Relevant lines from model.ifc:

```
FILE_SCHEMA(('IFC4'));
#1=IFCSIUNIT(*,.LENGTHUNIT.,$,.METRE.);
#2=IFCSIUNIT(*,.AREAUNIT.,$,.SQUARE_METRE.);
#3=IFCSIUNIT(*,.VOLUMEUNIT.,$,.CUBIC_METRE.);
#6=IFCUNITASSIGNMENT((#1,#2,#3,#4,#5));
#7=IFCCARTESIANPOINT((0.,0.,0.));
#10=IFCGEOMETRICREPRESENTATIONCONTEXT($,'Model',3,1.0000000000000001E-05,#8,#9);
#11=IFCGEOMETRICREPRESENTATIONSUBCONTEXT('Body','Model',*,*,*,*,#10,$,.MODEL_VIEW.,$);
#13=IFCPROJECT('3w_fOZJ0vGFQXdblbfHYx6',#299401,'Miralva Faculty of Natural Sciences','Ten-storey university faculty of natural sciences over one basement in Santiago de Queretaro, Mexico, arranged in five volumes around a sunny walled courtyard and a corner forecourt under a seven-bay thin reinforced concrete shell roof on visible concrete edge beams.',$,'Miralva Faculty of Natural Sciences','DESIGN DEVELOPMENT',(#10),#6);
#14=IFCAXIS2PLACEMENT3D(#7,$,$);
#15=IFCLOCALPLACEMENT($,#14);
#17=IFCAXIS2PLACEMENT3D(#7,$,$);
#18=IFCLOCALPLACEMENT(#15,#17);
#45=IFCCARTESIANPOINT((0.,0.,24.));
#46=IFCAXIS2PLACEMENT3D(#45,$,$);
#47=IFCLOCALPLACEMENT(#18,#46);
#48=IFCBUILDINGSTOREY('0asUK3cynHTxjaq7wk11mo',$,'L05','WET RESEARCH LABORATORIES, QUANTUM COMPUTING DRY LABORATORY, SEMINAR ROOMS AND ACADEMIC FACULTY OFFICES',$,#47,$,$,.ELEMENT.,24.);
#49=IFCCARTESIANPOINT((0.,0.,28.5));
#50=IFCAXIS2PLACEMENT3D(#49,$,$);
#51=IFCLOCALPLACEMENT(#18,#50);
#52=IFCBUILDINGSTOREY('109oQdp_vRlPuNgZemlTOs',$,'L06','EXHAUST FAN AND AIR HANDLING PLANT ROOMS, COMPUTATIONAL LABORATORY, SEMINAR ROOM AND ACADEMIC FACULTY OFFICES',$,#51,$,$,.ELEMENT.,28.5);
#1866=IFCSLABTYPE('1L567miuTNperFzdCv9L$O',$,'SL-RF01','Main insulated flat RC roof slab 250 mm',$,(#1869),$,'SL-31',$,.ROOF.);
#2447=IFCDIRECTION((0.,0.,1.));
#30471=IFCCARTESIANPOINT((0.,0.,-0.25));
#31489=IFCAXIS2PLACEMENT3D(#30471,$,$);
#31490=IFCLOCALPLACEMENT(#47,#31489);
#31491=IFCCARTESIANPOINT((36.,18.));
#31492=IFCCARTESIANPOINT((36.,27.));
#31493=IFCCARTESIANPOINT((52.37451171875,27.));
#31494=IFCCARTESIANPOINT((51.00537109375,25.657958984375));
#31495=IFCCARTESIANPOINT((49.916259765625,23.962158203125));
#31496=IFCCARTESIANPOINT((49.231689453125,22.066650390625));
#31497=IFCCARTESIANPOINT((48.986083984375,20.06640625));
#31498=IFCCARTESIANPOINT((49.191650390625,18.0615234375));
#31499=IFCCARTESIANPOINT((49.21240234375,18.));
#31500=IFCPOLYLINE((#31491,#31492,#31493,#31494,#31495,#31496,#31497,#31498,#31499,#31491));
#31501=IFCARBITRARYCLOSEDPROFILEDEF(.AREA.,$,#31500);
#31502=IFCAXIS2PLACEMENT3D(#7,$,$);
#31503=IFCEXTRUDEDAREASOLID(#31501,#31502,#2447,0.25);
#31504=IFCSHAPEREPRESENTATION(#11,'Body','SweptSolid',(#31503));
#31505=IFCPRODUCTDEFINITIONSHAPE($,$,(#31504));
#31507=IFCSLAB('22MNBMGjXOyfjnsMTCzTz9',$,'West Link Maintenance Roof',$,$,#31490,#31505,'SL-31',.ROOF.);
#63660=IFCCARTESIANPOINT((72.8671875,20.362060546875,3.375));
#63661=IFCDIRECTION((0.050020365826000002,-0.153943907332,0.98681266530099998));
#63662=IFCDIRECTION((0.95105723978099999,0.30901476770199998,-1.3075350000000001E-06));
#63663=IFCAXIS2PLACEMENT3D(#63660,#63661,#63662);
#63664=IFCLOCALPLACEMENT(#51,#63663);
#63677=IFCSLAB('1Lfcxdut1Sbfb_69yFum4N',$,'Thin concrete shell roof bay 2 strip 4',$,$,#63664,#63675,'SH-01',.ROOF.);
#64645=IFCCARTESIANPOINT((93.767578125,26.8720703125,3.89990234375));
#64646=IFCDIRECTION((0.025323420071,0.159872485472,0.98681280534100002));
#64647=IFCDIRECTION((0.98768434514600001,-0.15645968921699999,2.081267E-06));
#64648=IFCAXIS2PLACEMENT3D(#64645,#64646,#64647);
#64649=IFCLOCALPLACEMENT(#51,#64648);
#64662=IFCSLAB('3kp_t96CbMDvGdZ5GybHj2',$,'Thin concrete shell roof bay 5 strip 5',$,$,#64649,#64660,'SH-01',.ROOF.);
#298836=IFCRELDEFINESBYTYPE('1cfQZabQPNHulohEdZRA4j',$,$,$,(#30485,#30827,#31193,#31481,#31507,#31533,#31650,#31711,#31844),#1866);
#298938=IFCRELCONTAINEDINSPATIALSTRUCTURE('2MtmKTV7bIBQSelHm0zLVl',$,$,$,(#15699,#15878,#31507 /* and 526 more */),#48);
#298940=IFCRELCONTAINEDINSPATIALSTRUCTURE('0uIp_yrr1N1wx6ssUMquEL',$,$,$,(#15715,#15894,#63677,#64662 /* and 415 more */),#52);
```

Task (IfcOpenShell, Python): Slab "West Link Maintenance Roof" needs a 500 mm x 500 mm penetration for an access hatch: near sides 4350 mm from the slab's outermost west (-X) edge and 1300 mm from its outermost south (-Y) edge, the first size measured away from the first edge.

```python
import numpy as np
import ifcopenshell
import ifcopenshell.api.feature
import ifcopenshell.api.geometry
import ifcopenshell.api.root
import ifcopenshell.geom
import ifcopenshell.util.placement
import ifcopenshell.util.representation
import ifcopenshell.util.shape
import ifcopenshell.util.unit

model = ifcopenshell.open("model.ifc")
unit_scale = ifcopenshell.util.unit.calculate_unit_scale(model)
settings = ifcopenshell.geom.settings()


def volume(element):
    """Net volume in cubic metres, openings subtracted."""
    shape = ifcopenshell.geom.create_shape(settings, element)
    return ifcopenshell.util.shape.get_volume(shape.geometry)


slab = model.by_guid("22MNBMGjXOyfjnsMTCzTz9")
before = volume(slab)

# Extent in the slab's own axes, in metres. The edges named are its -X and -Y sides.
slab_shape = ifcopenshell.geom.create_shape(settings, slab)
vertices = ifcopenshell.util.shape.get_vertices(slab_shape.geometry)
x_min, y_min, bottom = vertices.min(axis=0)
top = vertices[:, 2].max()

opening = ifcopenshell.api.root.create_entity(model, ifc_class="IfcOpeningElement", name="Access hatch opening", predefined_type="OPENING")
context = ifcopenshell.util.representation.get_context(model, "Model", "Body", "MODEL_VIEW")
width, depth = 0.5, 0.5
outline = [(0.0, 0.0), (width, 0.0), (width, depth), (0.0, depth), (0.0, 0.0)]
# Overshoot both faces by 50 mm so the cut is clean.
shape = ifcopenshell.api.geometry.add_slab_representation(
    model, context=context, depth=top - bottom + 0.1, polyline=outline
)
ifcopenshell.api.geometry.assign_representation(model, product=opening, representation=shape)

matrix = ifcopenshell.util.placement.get_local_placement(slab.ObjectPlacement)
matrix[:, 3] = matrix @ np.append(np.array([x_min + 4.35, y_min + 1.3, bottom - 0.05]) / unit_scale, 1.0)
ifcopenshell.api.geometry.edit_object_placement(model, product=opening, matrix=matrix, is_si=False)
ifcopenshell.api.feature.add_feature(model, feature=opening, element=slab)

after = volume(slab)

print(f"slab volume {before:.3f} -> {after:.3f} m3")

model.write("model-out.ifc")
```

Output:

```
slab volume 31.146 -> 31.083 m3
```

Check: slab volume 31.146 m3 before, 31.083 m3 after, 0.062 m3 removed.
